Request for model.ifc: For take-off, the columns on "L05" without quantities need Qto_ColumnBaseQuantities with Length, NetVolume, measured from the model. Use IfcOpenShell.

First a look at what the model holds.

```python
import ifcopenshell
import ifcopenshell.util.element
import ifcopenshell.util.unit

model = ifcopenshell.open("model.ifc")
print(model.schema)
for unit_type in ("LENGTHUNIT", "AREAUNIT", "VOLUMEUNIT"):
    print(unit_type, ifcopenshell.util.unit.calculate_unit_scale(model, unit_type))
storey = next(s for s in model.by_type("IfcBuildingStorey") if s.Name == "L05")
columns = [e for e in ifcopenshell.util.element.get_decomposition(storey) if e.is_a("IfcColumn")]
for e in sorted(columns, key=lambda e: e.id()):
    print(e.id(), e.is_a(), e.Name, list(ifcopenshell.util.element.get_psets(e, qtos_only=True)), sep=" | ")
```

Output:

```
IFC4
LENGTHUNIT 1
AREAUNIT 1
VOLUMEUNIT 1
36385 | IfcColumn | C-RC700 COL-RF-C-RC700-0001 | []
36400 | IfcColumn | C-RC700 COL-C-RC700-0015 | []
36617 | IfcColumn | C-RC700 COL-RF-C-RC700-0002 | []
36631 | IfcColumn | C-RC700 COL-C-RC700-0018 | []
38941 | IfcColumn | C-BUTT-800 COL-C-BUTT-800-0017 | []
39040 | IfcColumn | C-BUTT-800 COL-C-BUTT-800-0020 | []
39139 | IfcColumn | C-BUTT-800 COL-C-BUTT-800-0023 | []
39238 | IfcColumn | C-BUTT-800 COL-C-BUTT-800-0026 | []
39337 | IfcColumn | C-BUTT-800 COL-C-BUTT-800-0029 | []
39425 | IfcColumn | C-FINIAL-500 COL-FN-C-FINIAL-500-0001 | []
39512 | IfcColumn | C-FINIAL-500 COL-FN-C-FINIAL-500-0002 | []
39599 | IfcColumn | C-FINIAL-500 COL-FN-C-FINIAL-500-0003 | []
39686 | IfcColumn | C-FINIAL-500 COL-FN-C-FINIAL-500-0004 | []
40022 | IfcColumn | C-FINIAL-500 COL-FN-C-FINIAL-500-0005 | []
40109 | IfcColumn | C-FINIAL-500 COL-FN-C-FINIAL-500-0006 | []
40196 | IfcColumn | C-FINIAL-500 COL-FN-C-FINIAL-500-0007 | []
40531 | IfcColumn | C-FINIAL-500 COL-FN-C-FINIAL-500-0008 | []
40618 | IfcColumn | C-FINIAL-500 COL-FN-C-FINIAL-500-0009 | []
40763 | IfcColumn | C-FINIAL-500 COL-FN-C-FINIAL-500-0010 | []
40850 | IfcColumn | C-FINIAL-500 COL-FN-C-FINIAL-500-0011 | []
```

```python
import ifcopenshell
import ifcopenshell.api.pset
import ifcopenshell.geom
import ifcopenshell.util.element
import ifcopenshell.util.shape
import ifcopenshell.util.unit

model = ifcopenshell.open("model.ifc")
unit_scale = ifcopenshell.util.unit.calculate_unit_scale(model)
volume_scale = ifcopenshell.util.unit.calculate_unit_scale(model, "VOLUMEUNIT")
settings = ifcopenshell.geom.settings()

storey = next(s for s in model.by_type("IfcBuildingStorey") if s.Name == "L05")
columns = [e for e in ifcopenshell.util.element.get_decomposition(storey) if e.is_a("IfcColumn")]

for e in sorted(columns, key=lambda e: e.id()):
    if ifcopenshell.util.element.get_psets(e, qtos_only=True, should_inherit=False):
        continue
    # Geometry comes back in metres, in the element's own axes.
    shape = ifcopenshell.geom.create_shape(settings, e)
    values = {
        "Length": ifcopenshell.util.shape.get_z(shape.geometry) / unit_scale,
        "NetVolume": ifcopenshell.util.shape.get_volume(shape.geometry) / volume_scale,
    }
    qto = ifcopenshell.api.pset.add_qto(model, product=e, name="Qto_ColumnBaseQuantities")
    ifcopenshell.api.pset.edit_qto(model, qto=qto, properties=values)
    print(e.id(), {k: round(v, 3) for k, v in values.items()})

model.write("model_rev.ifc")
```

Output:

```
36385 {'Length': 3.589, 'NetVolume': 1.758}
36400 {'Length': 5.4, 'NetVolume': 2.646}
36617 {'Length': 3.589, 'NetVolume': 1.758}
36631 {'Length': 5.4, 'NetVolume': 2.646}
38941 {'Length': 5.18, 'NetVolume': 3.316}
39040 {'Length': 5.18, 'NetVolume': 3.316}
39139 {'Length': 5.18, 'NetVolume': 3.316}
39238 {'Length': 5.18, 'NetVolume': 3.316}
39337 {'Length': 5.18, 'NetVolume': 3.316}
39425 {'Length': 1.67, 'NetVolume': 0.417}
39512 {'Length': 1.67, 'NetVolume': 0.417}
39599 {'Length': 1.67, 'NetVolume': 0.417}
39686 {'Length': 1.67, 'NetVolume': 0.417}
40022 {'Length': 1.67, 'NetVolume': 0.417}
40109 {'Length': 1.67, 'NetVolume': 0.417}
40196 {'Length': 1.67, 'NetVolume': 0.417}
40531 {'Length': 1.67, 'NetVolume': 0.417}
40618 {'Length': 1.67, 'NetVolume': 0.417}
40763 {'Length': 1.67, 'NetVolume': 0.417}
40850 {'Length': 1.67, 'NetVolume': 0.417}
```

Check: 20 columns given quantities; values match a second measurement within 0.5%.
